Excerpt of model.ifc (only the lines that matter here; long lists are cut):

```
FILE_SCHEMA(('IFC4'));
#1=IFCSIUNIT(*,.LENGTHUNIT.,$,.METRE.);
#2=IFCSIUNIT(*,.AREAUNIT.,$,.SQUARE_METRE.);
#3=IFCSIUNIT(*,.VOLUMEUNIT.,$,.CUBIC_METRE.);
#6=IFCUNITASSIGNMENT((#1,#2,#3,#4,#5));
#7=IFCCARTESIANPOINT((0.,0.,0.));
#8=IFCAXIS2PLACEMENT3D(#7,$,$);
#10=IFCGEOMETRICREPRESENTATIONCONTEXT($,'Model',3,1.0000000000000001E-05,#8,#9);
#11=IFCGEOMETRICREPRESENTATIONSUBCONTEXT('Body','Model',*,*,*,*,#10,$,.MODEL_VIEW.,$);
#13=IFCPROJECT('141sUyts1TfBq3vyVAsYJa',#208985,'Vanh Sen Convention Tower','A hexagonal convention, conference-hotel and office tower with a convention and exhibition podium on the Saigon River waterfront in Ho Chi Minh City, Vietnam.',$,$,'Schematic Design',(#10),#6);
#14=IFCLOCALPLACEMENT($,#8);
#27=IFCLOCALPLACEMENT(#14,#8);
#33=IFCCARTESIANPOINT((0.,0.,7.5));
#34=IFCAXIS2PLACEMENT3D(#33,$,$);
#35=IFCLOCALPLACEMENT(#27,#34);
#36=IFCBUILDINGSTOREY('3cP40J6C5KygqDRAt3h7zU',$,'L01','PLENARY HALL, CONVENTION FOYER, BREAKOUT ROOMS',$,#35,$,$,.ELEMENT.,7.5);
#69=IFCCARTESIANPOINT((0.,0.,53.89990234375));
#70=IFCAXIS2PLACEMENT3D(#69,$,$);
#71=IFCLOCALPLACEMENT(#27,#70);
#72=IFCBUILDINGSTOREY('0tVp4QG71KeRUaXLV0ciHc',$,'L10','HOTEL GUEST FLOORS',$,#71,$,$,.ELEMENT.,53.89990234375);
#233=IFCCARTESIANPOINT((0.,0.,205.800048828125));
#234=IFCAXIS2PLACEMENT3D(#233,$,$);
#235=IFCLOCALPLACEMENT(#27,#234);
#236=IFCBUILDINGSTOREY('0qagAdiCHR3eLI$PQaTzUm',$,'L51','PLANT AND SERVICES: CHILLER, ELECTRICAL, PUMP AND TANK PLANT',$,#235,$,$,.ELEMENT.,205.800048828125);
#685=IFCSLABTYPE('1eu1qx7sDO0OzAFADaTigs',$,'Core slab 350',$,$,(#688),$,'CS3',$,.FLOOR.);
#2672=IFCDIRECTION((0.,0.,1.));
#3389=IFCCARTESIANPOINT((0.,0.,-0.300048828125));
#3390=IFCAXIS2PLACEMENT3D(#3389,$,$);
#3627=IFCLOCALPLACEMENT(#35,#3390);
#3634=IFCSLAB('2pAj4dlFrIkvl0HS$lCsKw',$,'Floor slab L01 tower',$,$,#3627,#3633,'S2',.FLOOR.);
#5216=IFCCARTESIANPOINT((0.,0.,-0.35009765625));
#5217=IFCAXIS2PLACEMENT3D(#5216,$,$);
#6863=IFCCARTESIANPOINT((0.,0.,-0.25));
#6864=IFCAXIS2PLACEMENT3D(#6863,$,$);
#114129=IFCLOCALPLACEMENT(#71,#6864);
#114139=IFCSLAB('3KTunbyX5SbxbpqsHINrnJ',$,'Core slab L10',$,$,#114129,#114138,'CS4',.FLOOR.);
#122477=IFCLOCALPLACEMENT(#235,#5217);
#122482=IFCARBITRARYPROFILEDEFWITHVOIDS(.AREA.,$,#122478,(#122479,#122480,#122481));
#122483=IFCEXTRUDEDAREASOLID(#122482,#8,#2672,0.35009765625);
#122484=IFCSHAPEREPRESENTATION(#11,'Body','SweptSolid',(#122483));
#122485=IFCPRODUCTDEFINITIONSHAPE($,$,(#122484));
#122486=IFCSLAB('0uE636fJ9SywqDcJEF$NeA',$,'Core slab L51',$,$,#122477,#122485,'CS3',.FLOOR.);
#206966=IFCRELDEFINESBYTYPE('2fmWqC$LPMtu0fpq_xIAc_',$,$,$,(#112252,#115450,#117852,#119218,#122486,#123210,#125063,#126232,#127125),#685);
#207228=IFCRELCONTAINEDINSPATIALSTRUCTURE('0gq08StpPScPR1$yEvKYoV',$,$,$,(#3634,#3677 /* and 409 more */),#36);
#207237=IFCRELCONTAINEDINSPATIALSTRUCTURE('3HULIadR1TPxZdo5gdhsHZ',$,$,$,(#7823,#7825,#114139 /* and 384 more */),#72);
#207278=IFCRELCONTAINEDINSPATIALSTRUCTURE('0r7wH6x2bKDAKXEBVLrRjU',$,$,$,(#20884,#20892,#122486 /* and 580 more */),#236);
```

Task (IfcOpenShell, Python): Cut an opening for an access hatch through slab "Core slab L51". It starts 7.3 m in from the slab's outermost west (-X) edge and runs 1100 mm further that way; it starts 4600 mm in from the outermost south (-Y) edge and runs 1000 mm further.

```python
import numpy as np
import ifcopenshell
import ifcopenshell.api.feature
import ifcopenshell.api.geometry
import ifcopenshell.api.root
import ifcopenshell.geom
import ifcopenshell.util.placement
import ifcopenshell.util.representation
import ifcopenshell.util.shape
import ifcopenshell.util.unit

model = ifcopenshell.open("model.ifc")
unit_scale = ifcopenshell.util.unit.calculate_unit_scale(model)
settings = ifcopenshell.geom.settings()


def volume(element):
    """Net volume in cubic metres, openings subtracted."""
    shape = ifcopenshell.geom.create_shape(settings, element)
    return ifcopenshell.util.shape.get_volume(shape.geometry)


slab = model.by_id(122486)
before = volume(slab)

# Extent in the slab's own axes, in metres. The edges named are its -X and -Y sides.
slab_shape = ifcopenshell.geom.create_shape(settings, slab)
vertices = ifcopenshell.util.shape.get_vertices(slab_shape.geometry)
x_min, y_min, bottom = vertices.min(axis=0)
top = vertices[:, 2].max()

opening = ifcopenshell.api.root.create_entity(model, ifc_class="IfcOpeningElement", name="Access hatch opening", predefined_type="OPENING")
context = ifcopenshell.util.representation.get_context(model, "Model", "Body", "MODEL_VIEW")
width, depth = 1.1, 1
outline = [(0.0, 0.0), (width, 0.0), (width, depth), (0.0, depth), (0.0, 0.0)]
# Overshoot both faces by 50 mm so the cut is clean.
shape = ifcopenshell.api.geometry.add_slab_representation(
    model, context=context, depth=top - bottom + 0.1, polyline=outline
)
ifcopenshell.api.geometry.assign_representation(model, product=opening, representation=shape)

matrix = ifcopenshell.util.placement.get_local_placement(slab.ObjectPlacement)
matrix[:, 3] = matrix @ np.append(np.array([x_min + 7.3, y_min + 4.6, bottom - 0.05]) / unit_scale, 1.0)
ifcopenshell.api.geometry.edit_object_placement(model, product=opening, matrix=matrix, is_si=False)
ifcopenshell.api.feature.add_feature(model, feature=opening, element=slab)

after = volume(slab)

print(f"slab volume {before:.3f} -> {after:.3f} m3")

model.write("model-out.ifc")
```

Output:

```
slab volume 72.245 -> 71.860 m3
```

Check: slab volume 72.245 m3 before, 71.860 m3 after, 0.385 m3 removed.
